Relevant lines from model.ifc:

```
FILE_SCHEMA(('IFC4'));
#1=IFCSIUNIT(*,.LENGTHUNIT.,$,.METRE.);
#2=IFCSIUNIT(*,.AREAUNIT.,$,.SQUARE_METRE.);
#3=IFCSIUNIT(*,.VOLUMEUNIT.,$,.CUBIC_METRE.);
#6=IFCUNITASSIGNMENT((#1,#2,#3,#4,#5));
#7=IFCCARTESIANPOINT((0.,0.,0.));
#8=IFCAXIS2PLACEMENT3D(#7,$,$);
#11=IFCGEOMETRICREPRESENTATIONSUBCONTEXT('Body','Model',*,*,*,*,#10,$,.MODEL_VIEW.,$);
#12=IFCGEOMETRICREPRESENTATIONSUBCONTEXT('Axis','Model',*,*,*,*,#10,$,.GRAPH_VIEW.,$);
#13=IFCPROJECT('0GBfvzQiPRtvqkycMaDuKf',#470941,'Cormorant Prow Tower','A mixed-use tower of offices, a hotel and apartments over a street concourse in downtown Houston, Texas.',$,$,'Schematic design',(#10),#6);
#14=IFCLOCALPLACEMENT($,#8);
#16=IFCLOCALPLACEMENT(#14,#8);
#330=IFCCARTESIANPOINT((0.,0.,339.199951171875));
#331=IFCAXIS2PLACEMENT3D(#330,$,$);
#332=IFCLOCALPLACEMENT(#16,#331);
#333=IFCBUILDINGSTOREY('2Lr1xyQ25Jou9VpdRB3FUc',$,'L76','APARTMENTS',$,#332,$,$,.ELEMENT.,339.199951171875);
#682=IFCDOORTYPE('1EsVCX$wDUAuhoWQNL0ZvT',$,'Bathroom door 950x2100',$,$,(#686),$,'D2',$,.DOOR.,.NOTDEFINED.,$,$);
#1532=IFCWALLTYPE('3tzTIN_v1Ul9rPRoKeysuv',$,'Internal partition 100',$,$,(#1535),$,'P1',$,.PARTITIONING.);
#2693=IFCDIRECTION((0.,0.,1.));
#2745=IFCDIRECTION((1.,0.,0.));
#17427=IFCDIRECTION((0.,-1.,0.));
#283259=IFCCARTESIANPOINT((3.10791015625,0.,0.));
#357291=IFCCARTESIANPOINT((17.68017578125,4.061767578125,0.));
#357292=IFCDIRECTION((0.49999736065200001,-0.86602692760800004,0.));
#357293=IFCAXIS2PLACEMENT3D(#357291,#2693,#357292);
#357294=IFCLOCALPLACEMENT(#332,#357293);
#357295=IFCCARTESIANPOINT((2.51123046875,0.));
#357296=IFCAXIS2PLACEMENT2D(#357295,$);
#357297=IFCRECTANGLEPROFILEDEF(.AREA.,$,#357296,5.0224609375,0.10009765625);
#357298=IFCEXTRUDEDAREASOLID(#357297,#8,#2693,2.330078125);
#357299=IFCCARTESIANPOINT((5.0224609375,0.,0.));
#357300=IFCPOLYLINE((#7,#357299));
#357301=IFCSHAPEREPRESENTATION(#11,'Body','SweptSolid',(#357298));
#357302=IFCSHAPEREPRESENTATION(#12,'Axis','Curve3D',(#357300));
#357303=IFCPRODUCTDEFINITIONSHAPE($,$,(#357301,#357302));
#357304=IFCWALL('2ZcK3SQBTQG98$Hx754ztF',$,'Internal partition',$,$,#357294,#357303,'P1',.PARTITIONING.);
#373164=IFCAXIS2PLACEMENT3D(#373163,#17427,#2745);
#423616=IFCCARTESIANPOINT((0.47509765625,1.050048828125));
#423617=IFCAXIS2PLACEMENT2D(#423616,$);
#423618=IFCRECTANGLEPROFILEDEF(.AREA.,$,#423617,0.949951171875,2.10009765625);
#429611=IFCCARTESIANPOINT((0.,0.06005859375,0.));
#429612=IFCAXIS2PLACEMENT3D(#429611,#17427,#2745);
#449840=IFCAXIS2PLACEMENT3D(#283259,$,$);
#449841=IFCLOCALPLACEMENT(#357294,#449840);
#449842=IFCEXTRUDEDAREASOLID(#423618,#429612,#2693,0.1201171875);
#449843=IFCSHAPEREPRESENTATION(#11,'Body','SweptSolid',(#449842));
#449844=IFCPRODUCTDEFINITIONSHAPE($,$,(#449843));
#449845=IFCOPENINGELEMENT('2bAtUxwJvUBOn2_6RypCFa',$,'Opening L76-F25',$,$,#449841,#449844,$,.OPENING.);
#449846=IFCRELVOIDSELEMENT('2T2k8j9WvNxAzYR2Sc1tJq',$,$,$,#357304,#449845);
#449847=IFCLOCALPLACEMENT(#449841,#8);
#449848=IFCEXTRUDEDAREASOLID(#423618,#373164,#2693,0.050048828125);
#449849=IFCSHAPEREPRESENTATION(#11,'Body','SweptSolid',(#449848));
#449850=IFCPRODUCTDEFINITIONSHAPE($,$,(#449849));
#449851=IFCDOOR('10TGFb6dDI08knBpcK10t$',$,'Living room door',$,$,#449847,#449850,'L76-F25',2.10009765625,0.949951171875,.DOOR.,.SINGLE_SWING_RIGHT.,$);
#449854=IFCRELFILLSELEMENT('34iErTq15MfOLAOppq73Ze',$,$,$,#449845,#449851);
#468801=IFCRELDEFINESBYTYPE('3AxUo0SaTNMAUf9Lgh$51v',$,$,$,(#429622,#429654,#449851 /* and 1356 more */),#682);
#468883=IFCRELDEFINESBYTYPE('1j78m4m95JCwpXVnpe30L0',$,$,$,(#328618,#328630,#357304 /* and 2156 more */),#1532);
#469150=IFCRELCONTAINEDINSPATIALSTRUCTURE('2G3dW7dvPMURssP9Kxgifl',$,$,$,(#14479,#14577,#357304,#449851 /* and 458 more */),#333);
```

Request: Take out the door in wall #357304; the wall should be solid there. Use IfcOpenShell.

```python
import ifcopenshell
import ifcopenshell.api.feature
import ifcopenshell.api.root
import ifcopenshell.geom
import ifcopenshell.util.shape

model = ifcopenshell.open("model.ifc")
settings = ifcopenshell.geom.settings()


def volume(element):
    """Net volume in cubic metres, openings subtracted."""
    shape = ifcopenshell.geom.create_shape(settings, element)
    return ifcopenshell.util.shape.get_volume(shape.geometry)


door = model.by_guid("10TGFb6dDI08knBpcK10t$")
opening = door.FillsVoids[0].RelatingOpeningElement
wall = opening.VoidsElements[0].RelatingBuildingElement
before = volume(wall)

ifcopenshell.api.root.remove_product(model, product=door)
ifcopenshell.api.feature.remove_feature(model, feature=opening)

after = volume(wall)

print(f"wall volume {before:.3f} -> {after:.3f} m3")

model.write("model-out.ifc")
```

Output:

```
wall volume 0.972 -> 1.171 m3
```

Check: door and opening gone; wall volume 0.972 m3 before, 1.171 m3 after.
